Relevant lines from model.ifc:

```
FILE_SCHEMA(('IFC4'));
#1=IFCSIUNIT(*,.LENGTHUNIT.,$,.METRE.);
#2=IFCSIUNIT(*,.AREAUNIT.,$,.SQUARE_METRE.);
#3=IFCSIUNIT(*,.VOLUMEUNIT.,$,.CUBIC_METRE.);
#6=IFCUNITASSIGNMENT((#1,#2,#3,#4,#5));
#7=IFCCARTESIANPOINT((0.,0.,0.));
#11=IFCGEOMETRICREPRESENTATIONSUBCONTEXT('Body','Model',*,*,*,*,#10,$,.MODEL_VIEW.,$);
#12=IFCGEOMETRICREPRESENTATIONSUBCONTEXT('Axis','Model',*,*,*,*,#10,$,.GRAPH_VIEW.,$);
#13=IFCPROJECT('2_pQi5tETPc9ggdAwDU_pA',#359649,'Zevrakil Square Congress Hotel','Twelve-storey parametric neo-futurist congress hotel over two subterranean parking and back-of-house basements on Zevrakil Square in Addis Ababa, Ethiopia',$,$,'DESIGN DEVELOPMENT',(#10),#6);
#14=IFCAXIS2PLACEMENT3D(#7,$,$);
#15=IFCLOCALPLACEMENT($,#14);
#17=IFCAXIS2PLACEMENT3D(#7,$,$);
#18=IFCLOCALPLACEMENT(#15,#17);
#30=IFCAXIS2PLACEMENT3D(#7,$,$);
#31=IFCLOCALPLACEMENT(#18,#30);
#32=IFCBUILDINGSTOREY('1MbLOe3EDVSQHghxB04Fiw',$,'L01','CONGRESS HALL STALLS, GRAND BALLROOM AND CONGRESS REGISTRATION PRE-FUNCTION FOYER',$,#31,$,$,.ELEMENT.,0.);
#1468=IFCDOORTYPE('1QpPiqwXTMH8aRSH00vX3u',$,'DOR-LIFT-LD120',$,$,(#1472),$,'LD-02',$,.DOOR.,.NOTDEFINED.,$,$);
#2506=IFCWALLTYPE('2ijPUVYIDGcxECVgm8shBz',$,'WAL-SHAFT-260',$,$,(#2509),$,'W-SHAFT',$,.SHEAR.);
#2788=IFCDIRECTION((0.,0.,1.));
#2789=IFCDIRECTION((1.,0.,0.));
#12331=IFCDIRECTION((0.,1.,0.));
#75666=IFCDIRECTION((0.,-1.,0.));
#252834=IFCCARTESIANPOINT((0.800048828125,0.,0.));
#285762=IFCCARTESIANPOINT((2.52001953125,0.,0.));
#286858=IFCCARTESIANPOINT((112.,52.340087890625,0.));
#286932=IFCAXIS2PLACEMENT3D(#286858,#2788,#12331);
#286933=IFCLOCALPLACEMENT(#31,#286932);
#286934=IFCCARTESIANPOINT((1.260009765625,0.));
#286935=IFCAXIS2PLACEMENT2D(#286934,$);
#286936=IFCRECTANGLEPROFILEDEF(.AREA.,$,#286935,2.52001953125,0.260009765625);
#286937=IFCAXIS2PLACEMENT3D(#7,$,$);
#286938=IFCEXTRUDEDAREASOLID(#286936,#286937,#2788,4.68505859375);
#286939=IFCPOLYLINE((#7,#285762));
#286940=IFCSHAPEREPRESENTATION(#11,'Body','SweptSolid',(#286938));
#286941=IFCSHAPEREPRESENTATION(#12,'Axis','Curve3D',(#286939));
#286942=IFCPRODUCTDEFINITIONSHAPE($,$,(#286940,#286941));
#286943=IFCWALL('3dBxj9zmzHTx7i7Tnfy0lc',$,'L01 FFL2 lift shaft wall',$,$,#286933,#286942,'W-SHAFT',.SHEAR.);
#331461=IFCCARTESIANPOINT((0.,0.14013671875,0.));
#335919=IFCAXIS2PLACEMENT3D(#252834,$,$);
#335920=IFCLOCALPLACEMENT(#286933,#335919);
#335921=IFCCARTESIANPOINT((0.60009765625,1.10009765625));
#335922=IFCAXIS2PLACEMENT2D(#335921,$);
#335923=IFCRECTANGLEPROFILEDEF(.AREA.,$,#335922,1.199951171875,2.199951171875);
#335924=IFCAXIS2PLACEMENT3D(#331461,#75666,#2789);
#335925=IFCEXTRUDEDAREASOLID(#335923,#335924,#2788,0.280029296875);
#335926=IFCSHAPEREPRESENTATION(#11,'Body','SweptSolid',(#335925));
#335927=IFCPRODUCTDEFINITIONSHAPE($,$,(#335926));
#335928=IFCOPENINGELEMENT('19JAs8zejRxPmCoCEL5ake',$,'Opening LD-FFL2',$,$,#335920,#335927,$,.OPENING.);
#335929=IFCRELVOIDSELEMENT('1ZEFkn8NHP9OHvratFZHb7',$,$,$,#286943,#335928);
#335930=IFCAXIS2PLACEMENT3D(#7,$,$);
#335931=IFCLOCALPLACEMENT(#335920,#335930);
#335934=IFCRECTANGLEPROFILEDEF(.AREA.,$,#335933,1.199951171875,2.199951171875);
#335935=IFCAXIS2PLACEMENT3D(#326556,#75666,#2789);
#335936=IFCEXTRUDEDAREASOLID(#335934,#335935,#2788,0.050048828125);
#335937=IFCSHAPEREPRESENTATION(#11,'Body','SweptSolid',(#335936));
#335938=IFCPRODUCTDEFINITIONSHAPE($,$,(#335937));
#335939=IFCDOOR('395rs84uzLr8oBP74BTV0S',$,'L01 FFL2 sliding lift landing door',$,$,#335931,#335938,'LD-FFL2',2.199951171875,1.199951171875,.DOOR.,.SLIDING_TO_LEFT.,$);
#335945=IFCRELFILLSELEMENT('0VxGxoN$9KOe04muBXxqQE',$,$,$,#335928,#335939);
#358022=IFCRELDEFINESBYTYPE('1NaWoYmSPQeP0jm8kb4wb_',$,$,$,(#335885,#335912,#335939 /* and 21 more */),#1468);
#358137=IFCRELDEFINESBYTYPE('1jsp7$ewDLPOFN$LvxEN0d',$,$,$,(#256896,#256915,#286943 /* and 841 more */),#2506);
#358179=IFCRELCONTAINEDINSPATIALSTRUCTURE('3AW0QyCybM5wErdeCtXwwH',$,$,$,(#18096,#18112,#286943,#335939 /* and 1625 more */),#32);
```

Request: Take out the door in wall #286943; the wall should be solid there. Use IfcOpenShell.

```python
import ifcopenshell
import ifcopenshell.api.feature
import ifcopenshell.api.root
import ifcopenshell.geom
import ifcopenshell.util.shape

model = ifcopenshell.open("model.ifc")
settings = ifcopenshell.geom.settings()


def volume(element):
    """Net volume in cubic metres, openings subtracted."""
    shape = ifcopenshell.geom.create_shape(settings, element)
    return ifcopenshell.util.shape.get_volume(shape.geometry)


door = model.by_guid("395rs84uzLr8oBP74BTV0S")
opening = door.FillsVoids[0].RelatingOpeningElement
wall = opening.VoidsElements[0].RelatingBuildingElement
before = volume(wall)

ifcopenshell.api.root.remove_product(model, product=door)
ifcopenshell.api.feature.remove_feature(model, feature=opening)

after = volume(wall)

print(f"wall volume {before:.3f} -> {after:.3f} m3")

model.write("model_v2.ifc")
```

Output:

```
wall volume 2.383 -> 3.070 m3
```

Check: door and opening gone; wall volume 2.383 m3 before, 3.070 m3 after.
